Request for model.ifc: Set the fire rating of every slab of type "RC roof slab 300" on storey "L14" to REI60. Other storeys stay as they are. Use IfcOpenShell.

First a look at what the model holds.

```python
import ifcopenshell
import ifcopenshell.util.element

model = ifcopenshell.open("model.ifc")
print(model.schema)
storey = next(s for s in model.by_type("IfcBuildingStorey") if s.Name == "L14")
slabs = [e for e in ifcopenshell.util.element.get_decomposition(storey) if e.is_a("IfcSlab")]
seen = {}
for e in slabs:
    element_type = ifcopenshell.util.element.get_type(e)
    key = (element_type.Name if element_type != e and element_type else None, ifcopenshell.util.element.get_pset(e, "Pset_SlabCommon", "FireRating"))
    seen[key] = seen.get(key, 0) + 1
for (name, value), count in sorted(seen.items(), key=str):
    print(count, "x", name, "|", value)
```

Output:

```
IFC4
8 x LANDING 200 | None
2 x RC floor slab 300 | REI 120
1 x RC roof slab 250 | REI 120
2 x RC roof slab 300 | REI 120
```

```python
import ifcopenshell
import ifcopenshell.api.pset
import ifcopenshell.util.element

model = ifcopenshell.open("model.ifc")

storey = next(s for s in model.by_type("IfcBuildingStorey") if s.Name == "L14")
slabs = [e for e in ifcopenshell.util.element.get_decomposition(storey) if e.is_a("IfcSlab")]

count = 0
for e in slabs:
    element_type = ifcopenshell.util.element.get_type(e)
    if element_type in (None, e) or element_type.Name != "RC roof slab 300":
        continue
    # add_pset returns the element's existing set when there is one.
    pset = ifcopenshell.api.pset.add_pset(model, product=e, name="Pset_SlabCommon")
    ifcopenshell.api.pset.edit_pset(model, pset=pset, properties={"FireRating": "REI60"})
    count += 1

print(count, "slabs updated")

model.write("model_edited.ifc")
```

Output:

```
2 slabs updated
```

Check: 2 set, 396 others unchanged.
